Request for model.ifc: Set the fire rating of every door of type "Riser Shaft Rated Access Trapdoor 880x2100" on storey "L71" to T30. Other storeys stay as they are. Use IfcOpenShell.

First a look at what the model holds.

```python
import ifcopenshell
import ifcopenshell.util.element

model = ifcopenshell.open("model.ifc")
print(model.schema)
storey = next(s for s in model.by_type("IfcBuildingStorey") if s.Name == "L71")
doors = [e for e in ifcopenshell.util.element.get_decomposition(storey) if e.is_a("IfcDoor")]
seen = {}
for e in doors:
    element_type = ifcopenshell.util.element.get_type(e)
    key = (element_type.Name if element_type != e and element_type else None, ifcopenshell.util.element.get_pset(e, "Pset_DoorCommon", "FireRating"))
    seen[key] = seen.get(key, 0) + 1
for (name, value), count in sorted(seen.items(), key=str):
    print(count, "x", name, "|", value)
```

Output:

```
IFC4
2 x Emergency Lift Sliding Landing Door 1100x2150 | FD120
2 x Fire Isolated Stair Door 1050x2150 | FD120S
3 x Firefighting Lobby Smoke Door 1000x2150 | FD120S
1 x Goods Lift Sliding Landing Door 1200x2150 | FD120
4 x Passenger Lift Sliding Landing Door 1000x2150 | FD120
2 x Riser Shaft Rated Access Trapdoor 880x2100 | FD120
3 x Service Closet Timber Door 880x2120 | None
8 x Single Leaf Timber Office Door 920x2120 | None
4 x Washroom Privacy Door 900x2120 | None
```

```python
import ifcopenshell
import ifcopenshell.api.pset
import ifcopenshell.util.element

model = ifcopenshell.open("model.ifc")

storey = next(s for s in model.by_type("IfcBuildingStorey") if s.Name == "L71")
doors = [e for e in ifcopenshell.util.element.get_decomposition(storey) if e.is_a("IfcDoor")]

count = 0
for e in doors:
    element_type = ifcopenshell.util.element.get_type(e)
    if element_type in (None, e) or element_type.Name != "Riser Shaft Rated Access Trapdoor 880x2100":
        continue
    found = ifcopenshell.util.element.get_pset(e, "Pset_DoorCommon", should_inherit=False)
    if found:
        pset = model.by_id(found["id"])
        if len(ifcopenshell.util.element.get_elements_by_pset(pset)) > 1:
            pset = ifcopenshell.api.pset.unshare_pset(model, products=[e], pset=pset)[0]
    else:
        pset = ifcopenshell.api.pset.add_pset(model, product=e, name="Pset_DoorCommon")
    ifcopenshell.api.pset.edit_pset(model, pset=pset, properties={"FireRating": "T30"})
    count += 1

print(count, "doors updated")

model.write("model_edited.ifc")
```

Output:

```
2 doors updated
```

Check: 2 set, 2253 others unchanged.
